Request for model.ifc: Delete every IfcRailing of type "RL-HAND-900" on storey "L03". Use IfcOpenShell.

First a look at what the model holds.

```python
import ifcopenshell
import ifcopenshell.util.element

model = ifcopenshell.open("model.ifc")
print(model.schema)
storey = next(s for s in model.by_type("IfcBuildingStorey") if s.Name == "L03")
railings = [e for e in ifcopenshell.util.element.get_decomposition(storey) if e.is_a("IfcRailing")]
seen = {}
for e in railings:
    element_type = ifcopenshell.util.element.get_type(e)
    name = element_type.Name if element_type not in (None, e) else None
    seen[name] = seen.get(name, 0) + 1
for name, count in sorted(seen.items(), key=str):
    print(count, "x", name)
```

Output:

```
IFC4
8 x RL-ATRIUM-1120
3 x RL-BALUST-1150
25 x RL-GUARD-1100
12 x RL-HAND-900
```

```python
import ifcopenshell
import ifcopenshell.api.root
import ifcopenshell.util.element

model = ifcopenshell.open("model.ifc")

storey = next(s for s in model.by_type("IfcBuildingStorey") if s.Name == "L03")
railings = [e for e in ifcopenshell.util.element.get_decomposition(storey) if e.is_a("IfcRailing")]
targets = [e for e in railings if (t := ifcopenshell.util.element.get_type(e)) not in (None, e) and t.Name == "RL-HAND-900"]

for e in targets:
    ifcopenshell.api.root.remove_product(model, product=e)
print(len(targets), "removed")

model.write("model-out.ifc")
```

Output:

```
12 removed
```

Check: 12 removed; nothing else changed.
